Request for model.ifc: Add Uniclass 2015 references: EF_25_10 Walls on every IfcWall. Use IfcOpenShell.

First a look at what the model holds.

```python
import ifcopenshell

model = ifcopenshell.open("model.ifc")
print(model.schema)
print("classifications:", [c.Name for c in model.by_type("IfcClassification")])
for ifc_class in ("IfcDoor", "IfcRoof", "IfcStair", "IfcWall", "IfcWindow"):
    print(ifc_class, len(model.by_type(ifc_class)))
```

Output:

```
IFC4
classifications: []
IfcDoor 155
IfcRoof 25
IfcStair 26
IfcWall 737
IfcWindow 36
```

```python
import ifcopenshell
import ifcopenshell.api.classification

model = ifcopenshell.open("model.ifc")

system = ifcopenshell.api.classification.add_classification(model, classification="Uniclass 2015")

codes = {
    "IfcWall": ("EF_25_10", "Walls"),
}
for ifc_class, (code, name) in codes.items():
    products = model.by_type(ifc_class)
    ifcopenshell.api.classification.add_reference(
        model, products=products, classification=system, identification=code, name=name
    )
    print(code, len(products))

model.write("model_v2.ifc")
```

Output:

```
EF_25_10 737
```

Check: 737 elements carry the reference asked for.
